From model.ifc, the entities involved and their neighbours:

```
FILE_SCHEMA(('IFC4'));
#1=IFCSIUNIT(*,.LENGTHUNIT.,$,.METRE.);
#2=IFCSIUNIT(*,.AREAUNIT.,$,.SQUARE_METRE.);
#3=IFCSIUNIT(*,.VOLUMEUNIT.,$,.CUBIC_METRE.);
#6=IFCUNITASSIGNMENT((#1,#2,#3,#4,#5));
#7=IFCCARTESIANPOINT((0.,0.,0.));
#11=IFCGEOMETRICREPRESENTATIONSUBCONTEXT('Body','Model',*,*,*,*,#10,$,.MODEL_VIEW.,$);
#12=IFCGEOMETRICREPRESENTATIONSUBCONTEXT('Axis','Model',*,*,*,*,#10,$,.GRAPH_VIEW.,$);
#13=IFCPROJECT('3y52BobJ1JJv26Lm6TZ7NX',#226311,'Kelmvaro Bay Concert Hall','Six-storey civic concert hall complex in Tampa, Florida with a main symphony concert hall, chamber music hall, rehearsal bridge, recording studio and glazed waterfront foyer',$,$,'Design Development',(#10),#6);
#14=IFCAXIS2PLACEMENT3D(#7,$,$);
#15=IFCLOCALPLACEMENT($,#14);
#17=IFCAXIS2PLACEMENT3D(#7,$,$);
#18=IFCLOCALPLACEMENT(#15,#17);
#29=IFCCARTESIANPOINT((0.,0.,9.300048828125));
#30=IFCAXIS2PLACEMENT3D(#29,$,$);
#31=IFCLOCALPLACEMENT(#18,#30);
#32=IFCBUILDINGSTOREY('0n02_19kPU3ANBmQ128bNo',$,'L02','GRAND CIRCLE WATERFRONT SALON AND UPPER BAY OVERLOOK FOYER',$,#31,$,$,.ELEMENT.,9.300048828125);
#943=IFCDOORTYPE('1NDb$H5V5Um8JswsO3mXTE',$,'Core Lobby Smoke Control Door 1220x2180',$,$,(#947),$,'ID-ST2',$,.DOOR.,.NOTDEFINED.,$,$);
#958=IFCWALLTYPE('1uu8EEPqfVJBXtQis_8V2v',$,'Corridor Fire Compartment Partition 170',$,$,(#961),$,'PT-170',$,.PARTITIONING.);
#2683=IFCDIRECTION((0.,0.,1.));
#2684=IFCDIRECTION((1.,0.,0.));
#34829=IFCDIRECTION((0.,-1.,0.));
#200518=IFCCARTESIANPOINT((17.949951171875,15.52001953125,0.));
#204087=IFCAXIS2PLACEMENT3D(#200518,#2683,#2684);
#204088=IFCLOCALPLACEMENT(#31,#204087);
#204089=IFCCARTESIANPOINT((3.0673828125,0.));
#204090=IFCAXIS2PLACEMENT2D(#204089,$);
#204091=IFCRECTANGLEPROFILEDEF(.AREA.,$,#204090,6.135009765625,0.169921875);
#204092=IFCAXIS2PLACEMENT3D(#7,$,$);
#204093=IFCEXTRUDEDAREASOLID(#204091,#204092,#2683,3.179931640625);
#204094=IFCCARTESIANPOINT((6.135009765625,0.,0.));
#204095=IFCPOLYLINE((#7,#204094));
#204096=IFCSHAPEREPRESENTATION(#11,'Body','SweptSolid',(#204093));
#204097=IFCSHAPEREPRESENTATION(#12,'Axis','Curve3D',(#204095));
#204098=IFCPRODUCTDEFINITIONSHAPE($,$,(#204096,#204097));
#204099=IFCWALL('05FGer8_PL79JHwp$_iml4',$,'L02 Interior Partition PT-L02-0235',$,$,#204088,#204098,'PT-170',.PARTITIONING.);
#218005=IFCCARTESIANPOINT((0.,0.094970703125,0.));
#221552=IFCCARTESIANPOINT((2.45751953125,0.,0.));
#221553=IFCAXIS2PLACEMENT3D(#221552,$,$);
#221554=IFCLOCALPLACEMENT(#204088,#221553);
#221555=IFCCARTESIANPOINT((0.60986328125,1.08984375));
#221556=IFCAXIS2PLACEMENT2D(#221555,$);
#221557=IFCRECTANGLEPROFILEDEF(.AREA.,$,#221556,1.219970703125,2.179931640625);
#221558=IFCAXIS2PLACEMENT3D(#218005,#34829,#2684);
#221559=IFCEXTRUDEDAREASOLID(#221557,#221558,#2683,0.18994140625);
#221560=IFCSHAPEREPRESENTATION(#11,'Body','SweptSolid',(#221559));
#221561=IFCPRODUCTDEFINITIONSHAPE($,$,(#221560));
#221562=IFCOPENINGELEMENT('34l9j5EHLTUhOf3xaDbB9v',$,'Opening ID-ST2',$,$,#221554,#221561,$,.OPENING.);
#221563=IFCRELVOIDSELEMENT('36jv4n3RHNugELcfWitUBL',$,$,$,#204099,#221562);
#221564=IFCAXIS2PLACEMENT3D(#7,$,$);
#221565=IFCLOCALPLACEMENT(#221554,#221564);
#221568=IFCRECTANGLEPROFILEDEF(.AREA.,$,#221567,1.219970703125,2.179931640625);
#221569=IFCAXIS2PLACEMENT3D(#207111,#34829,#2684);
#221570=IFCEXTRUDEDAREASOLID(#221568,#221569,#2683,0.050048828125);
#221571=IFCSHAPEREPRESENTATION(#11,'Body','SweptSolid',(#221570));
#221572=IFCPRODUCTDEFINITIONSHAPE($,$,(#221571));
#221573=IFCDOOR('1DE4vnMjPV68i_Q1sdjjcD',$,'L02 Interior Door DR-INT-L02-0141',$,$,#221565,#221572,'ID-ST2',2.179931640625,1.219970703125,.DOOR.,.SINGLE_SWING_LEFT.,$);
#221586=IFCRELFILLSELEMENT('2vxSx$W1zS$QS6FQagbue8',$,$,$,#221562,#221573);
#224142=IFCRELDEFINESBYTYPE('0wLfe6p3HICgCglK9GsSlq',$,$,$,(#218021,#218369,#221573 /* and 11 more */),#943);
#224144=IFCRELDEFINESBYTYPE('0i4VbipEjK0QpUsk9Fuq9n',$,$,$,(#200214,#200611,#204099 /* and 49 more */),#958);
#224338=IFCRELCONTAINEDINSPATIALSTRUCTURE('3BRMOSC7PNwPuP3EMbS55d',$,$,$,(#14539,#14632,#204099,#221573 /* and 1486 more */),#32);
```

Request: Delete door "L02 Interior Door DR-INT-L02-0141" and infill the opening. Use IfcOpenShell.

```python
import ifcopenshell
import ifcopenshell.api.feature
import ifcopenshell.api.root
import ifcopenshell.geom
import ifcopenshell.util.shape

model = ifcopenshell.open("model.ifc")
settings = ifcopenshell.geom.settings()


def volume(element):
    """Net volume in cubic metres, openings subtracted."""
    shape = ifcopenshell.geom.create_shape(settings, element)
    return ifcopenshell.util.shape.get_volume(shape.geometry)


door = model.by_guid("1DE4vnMjPV68i_Q1sdjjcD")
opening = door.FillsVoids[0].RelatingOpeningElement
wall = opening.VoidsElements[0].RelatingBuildingElement
before = volume(wall)

ifcopenshell.api.root.remove_product(model, product=door)
ifcopenshell.api.feature.remove_feature(model, feature=opening)

after = volume(wall)

print(f"wall volume {before:.3f} -> {after:.3f} m3")

model.write("model_edited.ifc")
```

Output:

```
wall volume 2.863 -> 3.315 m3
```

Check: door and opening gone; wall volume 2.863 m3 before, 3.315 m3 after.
